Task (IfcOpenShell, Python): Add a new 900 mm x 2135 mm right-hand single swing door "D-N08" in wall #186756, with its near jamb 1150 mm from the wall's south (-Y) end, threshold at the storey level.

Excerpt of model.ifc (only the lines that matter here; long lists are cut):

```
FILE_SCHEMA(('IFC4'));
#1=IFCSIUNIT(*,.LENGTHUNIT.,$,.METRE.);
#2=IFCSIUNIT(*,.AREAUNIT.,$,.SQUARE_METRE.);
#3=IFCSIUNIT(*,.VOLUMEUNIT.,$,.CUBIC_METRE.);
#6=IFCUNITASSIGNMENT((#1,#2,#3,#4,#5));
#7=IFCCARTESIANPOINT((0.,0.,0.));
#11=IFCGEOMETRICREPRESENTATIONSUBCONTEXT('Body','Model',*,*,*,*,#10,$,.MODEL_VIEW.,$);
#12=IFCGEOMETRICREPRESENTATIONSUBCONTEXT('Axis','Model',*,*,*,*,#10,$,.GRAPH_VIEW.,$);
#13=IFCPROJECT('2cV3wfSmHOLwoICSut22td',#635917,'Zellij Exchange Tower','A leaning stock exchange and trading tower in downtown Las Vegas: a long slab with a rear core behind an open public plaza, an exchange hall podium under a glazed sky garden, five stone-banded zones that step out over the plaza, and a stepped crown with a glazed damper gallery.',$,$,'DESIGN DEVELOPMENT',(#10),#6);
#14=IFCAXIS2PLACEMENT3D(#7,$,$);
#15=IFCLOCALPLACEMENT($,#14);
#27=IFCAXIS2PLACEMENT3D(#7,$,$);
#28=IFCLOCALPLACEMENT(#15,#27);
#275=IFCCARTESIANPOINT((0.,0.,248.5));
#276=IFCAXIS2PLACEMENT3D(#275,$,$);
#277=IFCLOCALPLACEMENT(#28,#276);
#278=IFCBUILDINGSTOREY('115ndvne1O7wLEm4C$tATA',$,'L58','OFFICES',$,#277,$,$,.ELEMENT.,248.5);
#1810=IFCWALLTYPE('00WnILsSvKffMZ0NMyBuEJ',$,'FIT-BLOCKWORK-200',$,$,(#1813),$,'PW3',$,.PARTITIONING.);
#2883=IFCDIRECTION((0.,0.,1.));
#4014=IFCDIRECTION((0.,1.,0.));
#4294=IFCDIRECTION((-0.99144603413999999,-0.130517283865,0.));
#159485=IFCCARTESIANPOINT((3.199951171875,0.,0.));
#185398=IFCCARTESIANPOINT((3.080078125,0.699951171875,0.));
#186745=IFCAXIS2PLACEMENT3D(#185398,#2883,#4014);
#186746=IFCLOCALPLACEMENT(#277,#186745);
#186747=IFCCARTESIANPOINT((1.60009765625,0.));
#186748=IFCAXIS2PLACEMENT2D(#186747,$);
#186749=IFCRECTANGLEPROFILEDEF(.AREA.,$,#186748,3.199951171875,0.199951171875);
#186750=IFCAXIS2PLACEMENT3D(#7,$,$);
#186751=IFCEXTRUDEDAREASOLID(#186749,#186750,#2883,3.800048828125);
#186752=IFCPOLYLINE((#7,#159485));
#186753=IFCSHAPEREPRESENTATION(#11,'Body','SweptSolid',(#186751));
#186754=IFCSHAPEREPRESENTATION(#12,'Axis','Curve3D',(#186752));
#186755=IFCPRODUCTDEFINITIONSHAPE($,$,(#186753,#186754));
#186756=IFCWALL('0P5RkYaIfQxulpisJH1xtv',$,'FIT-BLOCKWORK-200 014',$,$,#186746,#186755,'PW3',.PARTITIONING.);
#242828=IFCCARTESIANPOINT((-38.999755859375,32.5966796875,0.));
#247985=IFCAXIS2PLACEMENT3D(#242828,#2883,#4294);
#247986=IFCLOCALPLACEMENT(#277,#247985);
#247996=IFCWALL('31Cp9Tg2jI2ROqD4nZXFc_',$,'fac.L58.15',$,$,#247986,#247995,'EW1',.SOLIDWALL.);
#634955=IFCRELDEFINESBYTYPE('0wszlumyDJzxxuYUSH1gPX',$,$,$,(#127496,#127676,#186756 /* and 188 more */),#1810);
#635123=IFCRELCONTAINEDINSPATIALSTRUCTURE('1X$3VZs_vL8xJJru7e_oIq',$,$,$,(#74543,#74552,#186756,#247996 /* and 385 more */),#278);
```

```python
import numpy as np
import ifcopenshell
import ifcopenshell.api.feature
import ifcopenshell.api.geometry
import ifcopenshell.api.root
import ifcopenshell.api.spatial
import ifcopenshell.geom
import ifcopenshell.util.element
import ifcopenshell.util.placement
import ifcopenshell.util.representation
import ifcopenshell.util.shape
import ifcopenshell.util.unit

model = ifcopenshell.open("model.ifc")
unit_scale = ifcopenshell.util.unit.calculate_unit_scale(model)
settings = ifcopenshell.geom.settings()


def volume(element):
    """Net volume in cubic metres, openings subtracted."""
    shape = ifcopenshell.geom.create_shape(settings, element)
    return ifcopenshell.util.shape.get_volume(shape.geometry)


wall = model.by_guid("0P5RkYaIfQxulpisJH1xtv")
storey = ifcopenshell.util.element.get_container(wall, ifc_class="IfcBuildingStorey")
context = ifcopenshell.util.representation.get_context(model, "Model", "Body", "MODEL_VIEW")
before = volume(wall)

width, height, from_end, sill = 0.9, 2.135, 1.15, 0.0  # metres

# The wall runs along its own X axis, and the end named is its -X end.
wall_shape = ifcopenshell.geom.create_shape(settings, wall)
x, y, z = ifcopenshell.util.shape.get_vertices(wall_shape.geometry).T
start = x.min() + from_end
face, thickness = float(y.min()), float(y.max() - y.min())
wall_matrix = ifcopenshell.util.placement.get_local_placement(wall.ObjectPlacement)
level = ifcopenshell.util.placement.get_local_placement(storey.ObjectPlacement)[2, 3]


def in_wall(x, y):
    """Placement at x, y metres in the wall's axes, at sill height."""
    matrix = wall_matrix.copy()
    matrix[:, 3] = wall_matrix @ np.array([x / unit_scale, y / unit_scale, 0.0, 1.0])
    matrix[2, 3] = level + sill / unit_scale
    return matrix


# Opening: a box that overshoots both wall faces by 50 mm.
opening = ifcopenshell.api.root.create_entity(model, ifc_class="IfcOpeningElement", predefined_type="OPENING")
box = ifcopenshell.api.geometry.add_wall_representation(
    model, context=context, length=width, height=height, thickness=thickness + 0.1
)
ifcopenshell.api.geometry.assign_representation(model, product=opening, representation=box)
ifcopenshell.api.geometry.edit_object_placement(model, product=opening, matrix=in_wall(start, face - 0.05), is_si=False)
ifcopenshell.api.feature.add_feature(model, feature=opening, element=wall)

door = ifcopenshell.api.root.create_entity(model, ifc_class="IfcDoor", name="D-N08", predefined_type="DOOR")
door.OverallWidth, door.OverallHeight = width / unit_scale, height / unit_scale
door.OperationType = "SINGLE_SWING_RIGHT"
body = ifcopenshell.api.geometry.add_door_representation(
    model,
    context=context,
    overall_width=door.OverallWidth,
    overall_height=door.OverallHeight,
    operation_type="SINGLE_SWING_RIGHT",
    lining_properties={"LiningDepth": thickness / unit_scale, "ThresholdDepth": thickness / unit_scale},
)
ifcopenshell.api.geometry.assign_representation(model, product=door, representation=body)
ifcopenshell.api.spatial.assign_container(model, products=[door], relating_structure=storey)
ifcopenshell.api.feature.add_filling(model, opening=opening, element=door)

# The lining spans the wall, so the door starts at the wall face.
ifcopenshell.api.geometry.edit_object_placement(model, product=door, matrix=in_wall(start, face), is_si=False)

after = volume(wall)

print(f"wall volume {before:.3f} -> {after:.3f} m3")

model.write("model_edited.ifc")
```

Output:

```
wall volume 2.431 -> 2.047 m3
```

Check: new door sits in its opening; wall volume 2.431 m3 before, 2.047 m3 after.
